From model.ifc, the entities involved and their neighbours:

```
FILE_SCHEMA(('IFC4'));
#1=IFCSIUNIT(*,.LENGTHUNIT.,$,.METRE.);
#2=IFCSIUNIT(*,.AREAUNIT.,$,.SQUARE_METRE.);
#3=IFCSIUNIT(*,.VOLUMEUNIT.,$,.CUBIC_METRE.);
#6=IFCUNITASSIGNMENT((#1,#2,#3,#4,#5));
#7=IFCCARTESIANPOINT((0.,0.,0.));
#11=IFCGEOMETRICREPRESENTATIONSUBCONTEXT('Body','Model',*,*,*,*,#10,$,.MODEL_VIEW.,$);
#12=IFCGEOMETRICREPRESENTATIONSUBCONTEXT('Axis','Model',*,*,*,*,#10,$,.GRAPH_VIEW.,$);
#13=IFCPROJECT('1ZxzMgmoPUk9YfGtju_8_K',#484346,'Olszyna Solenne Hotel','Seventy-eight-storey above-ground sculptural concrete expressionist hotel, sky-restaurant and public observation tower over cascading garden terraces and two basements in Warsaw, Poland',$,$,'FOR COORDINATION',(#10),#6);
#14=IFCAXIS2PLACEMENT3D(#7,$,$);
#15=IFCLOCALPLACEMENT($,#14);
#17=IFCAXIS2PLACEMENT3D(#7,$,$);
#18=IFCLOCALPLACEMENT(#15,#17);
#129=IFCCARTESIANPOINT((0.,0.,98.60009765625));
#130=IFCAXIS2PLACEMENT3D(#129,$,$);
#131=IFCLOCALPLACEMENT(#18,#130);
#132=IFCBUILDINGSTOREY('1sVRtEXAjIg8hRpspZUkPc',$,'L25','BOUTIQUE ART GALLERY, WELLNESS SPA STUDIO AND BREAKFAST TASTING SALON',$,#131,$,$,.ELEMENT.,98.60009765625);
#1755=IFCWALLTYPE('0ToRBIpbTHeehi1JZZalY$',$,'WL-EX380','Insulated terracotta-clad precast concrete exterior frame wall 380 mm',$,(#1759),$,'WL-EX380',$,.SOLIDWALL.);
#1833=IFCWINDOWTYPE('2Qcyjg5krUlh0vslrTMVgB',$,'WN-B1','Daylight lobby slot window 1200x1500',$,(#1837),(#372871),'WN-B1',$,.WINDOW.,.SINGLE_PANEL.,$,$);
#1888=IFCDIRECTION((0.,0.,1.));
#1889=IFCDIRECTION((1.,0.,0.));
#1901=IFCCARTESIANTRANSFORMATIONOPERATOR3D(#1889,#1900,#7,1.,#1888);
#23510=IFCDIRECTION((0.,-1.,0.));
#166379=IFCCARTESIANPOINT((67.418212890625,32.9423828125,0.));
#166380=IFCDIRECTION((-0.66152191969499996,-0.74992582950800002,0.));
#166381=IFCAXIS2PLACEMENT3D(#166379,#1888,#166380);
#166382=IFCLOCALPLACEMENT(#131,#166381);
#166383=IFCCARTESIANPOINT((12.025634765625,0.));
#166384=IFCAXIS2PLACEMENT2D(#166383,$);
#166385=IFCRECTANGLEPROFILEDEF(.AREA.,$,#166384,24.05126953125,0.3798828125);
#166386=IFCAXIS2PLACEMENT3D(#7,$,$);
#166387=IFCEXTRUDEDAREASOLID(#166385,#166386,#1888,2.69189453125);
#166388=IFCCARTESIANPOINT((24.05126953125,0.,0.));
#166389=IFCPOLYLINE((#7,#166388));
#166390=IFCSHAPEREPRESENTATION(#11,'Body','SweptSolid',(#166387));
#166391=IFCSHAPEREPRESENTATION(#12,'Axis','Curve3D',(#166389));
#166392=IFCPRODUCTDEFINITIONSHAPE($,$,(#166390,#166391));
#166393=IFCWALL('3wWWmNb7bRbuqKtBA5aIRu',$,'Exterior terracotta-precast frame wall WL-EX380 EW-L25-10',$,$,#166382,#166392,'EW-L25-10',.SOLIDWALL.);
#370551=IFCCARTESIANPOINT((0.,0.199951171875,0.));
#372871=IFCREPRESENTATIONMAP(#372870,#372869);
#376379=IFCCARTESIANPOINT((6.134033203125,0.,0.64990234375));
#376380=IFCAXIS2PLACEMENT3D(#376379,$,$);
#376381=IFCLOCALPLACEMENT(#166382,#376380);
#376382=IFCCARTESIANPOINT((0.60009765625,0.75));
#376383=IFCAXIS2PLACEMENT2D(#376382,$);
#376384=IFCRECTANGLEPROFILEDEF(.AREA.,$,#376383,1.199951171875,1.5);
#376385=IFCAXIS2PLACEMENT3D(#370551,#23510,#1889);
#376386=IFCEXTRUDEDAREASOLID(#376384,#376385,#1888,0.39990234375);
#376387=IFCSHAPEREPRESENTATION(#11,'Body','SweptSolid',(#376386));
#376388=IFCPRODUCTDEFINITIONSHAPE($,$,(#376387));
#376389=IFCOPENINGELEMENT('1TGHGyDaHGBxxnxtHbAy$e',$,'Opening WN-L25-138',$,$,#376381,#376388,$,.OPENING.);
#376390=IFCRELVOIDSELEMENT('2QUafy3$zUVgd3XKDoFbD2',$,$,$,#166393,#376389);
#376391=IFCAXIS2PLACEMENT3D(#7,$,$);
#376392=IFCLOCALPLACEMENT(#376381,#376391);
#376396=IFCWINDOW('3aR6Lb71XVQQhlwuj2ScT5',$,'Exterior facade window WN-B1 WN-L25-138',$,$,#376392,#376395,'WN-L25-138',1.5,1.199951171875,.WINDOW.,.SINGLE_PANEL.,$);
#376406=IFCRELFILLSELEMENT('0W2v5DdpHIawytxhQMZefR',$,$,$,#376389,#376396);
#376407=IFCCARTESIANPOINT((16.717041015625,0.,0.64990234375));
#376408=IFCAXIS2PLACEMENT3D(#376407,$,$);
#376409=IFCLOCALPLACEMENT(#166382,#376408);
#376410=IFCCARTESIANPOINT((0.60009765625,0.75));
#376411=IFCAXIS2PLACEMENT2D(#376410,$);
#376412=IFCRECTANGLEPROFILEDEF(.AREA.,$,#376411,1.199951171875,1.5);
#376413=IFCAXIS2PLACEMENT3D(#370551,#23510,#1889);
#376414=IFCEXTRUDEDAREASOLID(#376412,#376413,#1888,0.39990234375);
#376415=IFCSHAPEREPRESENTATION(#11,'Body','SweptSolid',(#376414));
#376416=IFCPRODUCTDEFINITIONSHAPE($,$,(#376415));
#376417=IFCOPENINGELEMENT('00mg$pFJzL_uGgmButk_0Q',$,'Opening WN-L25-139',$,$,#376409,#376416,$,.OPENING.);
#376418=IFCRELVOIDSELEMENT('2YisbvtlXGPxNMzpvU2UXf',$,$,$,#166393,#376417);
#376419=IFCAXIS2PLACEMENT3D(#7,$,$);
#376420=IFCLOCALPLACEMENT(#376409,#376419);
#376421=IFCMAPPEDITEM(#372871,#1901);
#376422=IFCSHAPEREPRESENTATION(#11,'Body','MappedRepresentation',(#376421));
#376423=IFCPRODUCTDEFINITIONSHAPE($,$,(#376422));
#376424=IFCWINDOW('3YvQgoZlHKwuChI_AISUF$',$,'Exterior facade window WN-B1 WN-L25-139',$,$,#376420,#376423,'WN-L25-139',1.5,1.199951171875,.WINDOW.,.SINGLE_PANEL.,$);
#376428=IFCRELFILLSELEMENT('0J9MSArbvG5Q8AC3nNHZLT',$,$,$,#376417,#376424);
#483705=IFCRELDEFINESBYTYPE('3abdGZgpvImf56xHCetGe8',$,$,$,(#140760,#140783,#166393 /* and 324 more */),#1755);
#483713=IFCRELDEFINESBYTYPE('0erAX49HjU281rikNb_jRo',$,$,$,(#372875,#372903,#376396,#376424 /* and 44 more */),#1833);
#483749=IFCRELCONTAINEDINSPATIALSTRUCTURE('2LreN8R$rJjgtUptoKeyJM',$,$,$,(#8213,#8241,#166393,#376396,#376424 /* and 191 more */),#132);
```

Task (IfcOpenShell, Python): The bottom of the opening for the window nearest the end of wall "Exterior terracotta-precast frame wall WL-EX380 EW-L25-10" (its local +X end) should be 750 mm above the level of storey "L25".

```python
import numpy as np
import ifcopenshell
import ifcopenshell.api.geometry
import ifcopenshell.geom
import ifcopenshell.util.element
import ifcopenshell.util.placement
import ifcopenshell.util.shape
import ifcopenshell.util.unit

model = ifcopenshell.open("model.ifc")
unit_scale = ifcopenshell.util.unit.calculate_unit_scale(model)

window = model.by_id(376424)
opening = window.FillsVoids[0].RelatingOpeningElement
storey = ifcopenshell.util.element.get_container(window, ifc_class="IfcBuildingStorey")
level = ifcopenshell.util.placement.get_local_placement(storey.ObjectPlacement)[2, 3]

# The opening's origin need not be at the sill, so measure its lowest point.
shape = ifcopenshell.geom.create_shape(ifcopenshell.geom.settings(), opening)
bottom = ifcopenshell.util.shape.get_shape_bottom_elevation(shape, shape.geometry) / unit_scale
dz = level + 0.75 - bottom

shift = np.array([0.0, 0.0, dz])
# The window is placed relative to its opening, so it follows when the opening moves.
matrix = ifcopenshell.util.placement.get_local_placement(opening.ObjectPlacement)
matrix[:3, 3] += shift
ifcopenshell.api.geometry.edit_object_placement(
    model, product=opening, matrix=matrix, is_si=False, should_transform_children=True
)

print(f"moved by {dz * unit_scale:+.3f} m")

model.write("model_v2.ifc")
```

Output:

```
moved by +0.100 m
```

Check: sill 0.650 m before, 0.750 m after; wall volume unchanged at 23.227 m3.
